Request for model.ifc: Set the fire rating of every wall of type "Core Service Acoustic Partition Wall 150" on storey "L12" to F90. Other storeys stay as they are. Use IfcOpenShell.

First a look at what the model holds.

```python
import ifcopenshell
import ifcopenshell.util.element

model = ifcopenshell.open("model.ifc")
print(model.schema)
storey = next(s for s in model.by_type("IfcBuildingStorey") if s.Name == "L12")
walls = [e for e in ifcopenshell.util.element.get_decomposition(storey) if e.is_a("IfcWall")]
seen = {}
for e in walls:
    element_type = ifcopenshell.util.element.get_type(e)
    key = (element_type.Name if element_type != e and element_type else None, ifcopenshell.util.element.get_pset(e, "Pset_WallCommon", "FireRating"))
    seen[key] = seen.get(key, 0) + 1
for (name, value), count in sorted(seen.items(), key=str):
    print(count, "x", name, "|", value)
```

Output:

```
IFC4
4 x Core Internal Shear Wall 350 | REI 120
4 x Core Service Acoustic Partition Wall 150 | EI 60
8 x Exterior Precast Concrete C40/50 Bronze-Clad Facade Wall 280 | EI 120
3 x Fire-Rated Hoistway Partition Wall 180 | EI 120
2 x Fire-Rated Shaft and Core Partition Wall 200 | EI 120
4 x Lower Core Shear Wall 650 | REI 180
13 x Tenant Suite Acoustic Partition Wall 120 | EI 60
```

```python
import ifcopenshell
import ifcopenshell.api.pset
import ifcopenshell.util.element

model = ifcopenshell.open("model.ifc")

storey = next(s for s in model.by_type("IfcBuildingStorey") if s.Name == "L12")
walls = [e for e in ifcopenshell.util.element.get_decomposition(storey) if e.is_a("IfcWall")]

count = 0
for e in walls:
    element_type = ifcopenshell.util.element.get_type(e)
    if element_type in (None, e) or element_type.Name != "Core Service Acoustic Partition Wall 150":
        continue
    # add_pset returns the element's existing set when there is one.
    pset = ifcopenshell.api.pset.add_pset(model, product=e, name="Pset_WallCommon")
    ifcopenshell.api.pset.edit_pset(model, pset=pset, properties={"FireRating": "F90"})
    count += 1

print(count, "walls updated")

model.write("model-out.ifc")
```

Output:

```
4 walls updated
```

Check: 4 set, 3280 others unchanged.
